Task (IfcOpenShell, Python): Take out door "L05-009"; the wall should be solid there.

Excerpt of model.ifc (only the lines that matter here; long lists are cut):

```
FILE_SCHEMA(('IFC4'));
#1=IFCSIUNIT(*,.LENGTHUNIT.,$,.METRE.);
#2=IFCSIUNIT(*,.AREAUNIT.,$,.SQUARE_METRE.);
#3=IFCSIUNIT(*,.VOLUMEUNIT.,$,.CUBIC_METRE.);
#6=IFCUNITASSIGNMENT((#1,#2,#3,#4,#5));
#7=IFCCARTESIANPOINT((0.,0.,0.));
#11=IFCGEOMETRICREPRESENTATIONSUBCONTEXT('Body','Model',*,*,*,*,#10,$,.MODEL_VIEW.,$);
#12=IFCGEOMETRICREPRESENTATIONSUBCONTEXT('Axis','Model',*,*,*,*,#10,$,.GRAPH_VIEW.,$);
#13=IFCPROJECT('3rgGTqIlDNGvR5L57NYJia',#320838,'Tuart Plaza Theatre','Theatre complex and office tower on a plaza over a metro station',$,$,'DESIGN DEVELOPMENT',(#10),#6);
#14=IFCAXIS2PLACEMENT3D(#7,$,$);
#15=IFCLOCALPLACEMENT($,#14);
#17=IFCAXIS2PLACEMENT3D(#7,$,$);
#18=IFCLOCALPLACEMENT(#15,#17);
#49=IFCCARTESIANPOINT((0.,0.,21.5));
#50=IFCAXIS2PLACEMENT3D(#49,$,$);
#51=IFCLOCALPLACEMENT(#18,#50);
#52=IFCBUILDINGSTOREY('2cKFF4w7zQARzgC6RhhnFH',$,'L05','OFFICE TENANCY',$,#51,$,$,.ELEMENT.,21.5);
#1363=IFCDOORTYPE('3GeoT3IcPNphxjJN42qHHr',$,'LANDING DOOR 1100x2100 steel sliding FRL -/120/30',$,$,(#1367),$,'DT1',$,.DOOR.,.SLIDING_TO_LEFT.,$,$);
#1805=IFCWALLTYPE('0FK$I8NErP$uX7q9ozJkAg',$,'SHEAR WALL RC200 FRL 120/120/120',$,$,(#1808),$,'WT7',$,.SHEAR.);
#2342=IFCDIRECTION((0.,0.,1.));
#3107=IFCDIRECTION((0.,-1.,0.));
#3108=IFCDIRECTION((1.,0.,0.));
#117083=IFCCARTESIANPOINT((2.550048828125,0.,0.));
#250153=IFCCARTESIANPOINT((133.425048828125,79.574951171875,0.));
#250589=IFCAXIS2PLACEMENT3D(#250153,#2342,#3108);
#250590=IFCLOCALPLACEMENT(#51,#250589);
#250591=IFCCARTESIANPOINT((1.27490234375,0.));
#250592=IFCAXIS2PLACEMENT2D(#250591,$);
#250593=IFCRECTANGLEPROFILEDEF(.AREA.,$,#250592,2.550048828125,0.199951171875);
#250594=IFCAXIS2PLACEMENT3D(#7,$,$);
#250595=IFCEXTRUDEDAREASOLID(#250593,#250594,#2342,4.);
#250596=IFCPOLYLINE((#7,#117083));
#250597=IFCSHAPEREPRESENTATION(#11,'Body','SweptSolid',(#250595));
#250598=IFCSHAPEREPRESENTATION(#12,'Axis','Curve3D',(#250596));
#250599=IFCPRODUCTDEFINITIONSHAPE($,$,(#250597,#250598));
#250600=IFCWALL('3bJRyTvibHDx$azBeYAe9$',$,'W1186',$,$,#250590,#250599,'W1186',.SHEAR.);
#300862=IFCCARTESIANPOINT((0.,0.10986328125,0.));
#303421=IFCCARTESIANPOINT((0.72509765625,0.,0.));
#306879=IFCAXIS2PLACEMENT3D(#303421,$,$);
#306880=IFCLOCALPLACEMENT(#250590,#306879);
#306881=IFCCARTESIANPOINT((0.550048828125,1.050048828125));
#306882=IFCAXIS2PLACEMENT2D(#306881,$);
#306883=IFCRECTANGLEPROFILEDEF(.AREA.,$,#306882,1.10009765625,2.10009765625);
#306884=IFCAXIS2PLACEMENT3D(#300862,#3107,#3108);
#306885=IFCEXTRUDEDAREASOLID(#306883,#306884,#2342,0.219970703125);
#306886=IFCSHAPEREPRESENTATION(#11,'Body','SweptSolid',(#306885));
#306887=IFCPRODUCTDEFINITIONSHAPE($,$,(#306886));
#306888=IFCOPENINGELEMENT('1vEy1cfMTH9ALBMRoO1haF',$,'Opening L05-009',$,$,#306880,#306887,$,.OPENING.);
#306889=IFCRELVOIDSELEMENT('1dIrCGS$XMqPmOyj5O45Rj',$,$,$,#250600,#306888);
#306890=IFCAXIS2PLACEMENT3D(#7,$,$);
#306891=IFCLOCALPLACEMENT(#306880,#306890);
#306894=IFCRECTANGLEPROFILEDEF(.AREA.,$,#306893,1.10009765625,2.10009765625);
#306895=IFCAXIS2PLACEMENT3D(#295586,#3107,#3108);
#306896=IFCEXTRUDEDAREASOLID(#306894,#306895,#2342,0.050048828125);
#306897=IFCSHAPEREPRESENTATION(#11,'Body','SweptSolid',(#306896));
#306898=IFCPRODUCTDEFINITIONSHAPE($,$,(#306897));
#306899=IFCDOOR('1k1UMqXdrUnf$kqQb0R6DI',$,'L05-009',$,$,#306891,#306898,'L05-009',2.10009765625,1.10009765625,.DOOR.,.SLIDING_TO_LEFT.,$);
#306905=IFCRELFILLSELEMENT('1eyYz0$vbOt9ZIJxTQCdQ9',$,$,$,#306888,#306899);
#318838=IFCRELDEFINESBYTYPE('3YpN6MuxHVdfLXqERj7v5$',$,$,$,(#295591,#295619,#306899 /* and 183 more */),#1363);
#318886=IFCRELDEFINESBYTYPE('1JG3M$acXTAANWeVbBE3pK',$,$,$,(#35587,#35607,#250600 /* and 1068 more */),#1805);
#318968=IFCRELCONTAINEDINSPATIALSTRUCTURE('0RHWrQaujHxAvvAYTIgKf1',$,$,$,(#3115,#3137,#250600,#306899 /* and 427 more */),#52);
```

```python
import ifcopenshell
import ifcopenshell.api.feature
import ifcopenshell.api.root
import ifcopenshell.geom
import ifcopenshell.util.shape

model = ifcopenshell.open("model.ifc")
settings = ifcopenshell.geom.settings()


def volume(element):
    """Net volume in cubic metres, openings subtracted."""
    shape = ifcopenshell.geom.create_shape(settings, element)
    return ifcopenshell.util.shape.get_volume(shape.geometry)


door = model.by_id(306899)
opening = door.FillsVoids[0].RelatingOpeningElement
wall = opening.VoidsElements[0].RelatingBuildingElement
before = volume(wall)

ifcopenshell.api.root.remove_product(model, product=door)
ifcopenshell.api.feature.remove_feature(model, feature=opening)

after = volume(wall)

print(f"wall volume {before:.3f} -> {after:.3f} m3")

model.write("model_updated.ifc")
```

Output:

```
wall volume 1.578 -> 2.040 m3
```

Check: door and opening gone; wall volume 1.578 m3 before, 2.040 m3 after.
